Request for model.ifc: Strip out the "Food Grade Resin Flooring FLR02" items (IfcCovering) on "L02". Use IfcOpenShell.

First a look at what the model holds.

```python
import ifcopenshell
import ifcopenshell.util.element

model = ifcopenshell.open("model.ifc")
print(model.schema)
storey = next(s for s in model.by_type("IfcBuildingStorey") if s.Name == "L02")
coverings = [e for e in ifcopenshell.util.element.get_decomposition(storey) if e.is_a("IfcCovering")]
seen = {}
for e in coverings:
    element_type = ifcopenshell.util.element.get_type(e)
    name = element_type.Name if element_type not in (None, e) else None
    seen[name] = seen.get(name, 0) + 1
for name, count in sorted(seen.items(), key=str):
    print(count, "x", name)
```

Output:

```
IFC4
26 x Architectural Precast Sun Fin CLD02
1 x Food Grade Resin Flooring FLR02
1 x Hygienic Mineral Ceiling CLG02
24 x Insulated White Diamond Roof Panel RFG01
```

```python
import ifcopenshell
import ifcopenshell.api.root
import ifcopenshell.util.element

model = ifcopenshell.open("model.ifc")

storey = next(s for s in model.by_type("IfcBuildingStorey") if s.Name == "L02")
coverings = [e for e in ifcopenshell.util.element.get_decomposition(storey) if e.is_a("IfcCovering")]
targets = [e for e in coverings if (t := ifcopenshell.util.element.get_type(e)) not in (None, e) and t.Name == "Food Grade Resin Flooring FLR02"]

for e in targets:
    ifcopenshell.api.root.remove_product(model, product=e)
print(len(targets), "removed")

model.write("model-out.ifc")
```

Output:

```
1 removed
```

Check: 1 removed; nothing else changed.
